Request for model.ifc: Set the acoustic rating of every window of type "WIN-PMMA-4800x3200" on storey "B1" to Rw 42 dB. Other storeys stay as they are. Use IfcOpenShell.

First a look at what the model holds.

```python
import ifcopenshell
import ifcopenshell.util.element

model = ifcopenshell.open("model.ifc")
print(model.schema)
storey = next(s for s in model.by_type("IfcBuildingStorey") if s.Name == "B1")
windows = [e for e in ifcopenshell.util.element.get_decomposition(storey) if e.is_a("IfcWindow")]
seen = {}
for e in windows:
    element_type = ifcopenshell.util.element.get_type(e)
    key = (element_type.Name if element_type != e and element_type else None, ifcopenshell.util.element.get_pset(e, "Pset_WindowCommon", "AcousticRating"))
    seen[key] = seen.get(key, 0) + 1
for (name, value), count in sorted(seen.items(), key=str):
    print(count, "x", name, "|", value)
```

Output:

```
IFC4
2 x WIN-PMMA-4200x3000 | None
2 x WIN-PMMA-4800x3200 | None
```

```python
import ifcopenshell
import ifcopenshell.api.pset
import ifcopenshell.util.element

model = ifcopenshell.open("model.ifc")

storey = next(s for s in model.by_type("IfcBuildingStorey") if s.Name == "B1")
windows = [e for e in ifcopenshell.util.element.get_decomposition(storey) if e.is_a("IfcWindow")]

count = 0
for e in windows:
    element_type = ifcopenshell.util.element.get_type(e)
    if element_type in (None, e) or element_type.Name != "WIN-PMMA-4800x3200":
        continue
    # add_pset returns the element's existing set when there is one.
    pset = ifcopenshell.api.pset.add_pset(model, product=e, name="Pset_WindowCommon")
    ifcopenshell.api.pset.edit_pset(model, pset=pset, properties={"AcousticRating": "Rw 42 dB"})
    count += 1

print(count, "windows updated")

model.write("model-out.ifc")
```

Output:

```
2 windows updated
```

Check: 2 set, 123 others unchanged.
